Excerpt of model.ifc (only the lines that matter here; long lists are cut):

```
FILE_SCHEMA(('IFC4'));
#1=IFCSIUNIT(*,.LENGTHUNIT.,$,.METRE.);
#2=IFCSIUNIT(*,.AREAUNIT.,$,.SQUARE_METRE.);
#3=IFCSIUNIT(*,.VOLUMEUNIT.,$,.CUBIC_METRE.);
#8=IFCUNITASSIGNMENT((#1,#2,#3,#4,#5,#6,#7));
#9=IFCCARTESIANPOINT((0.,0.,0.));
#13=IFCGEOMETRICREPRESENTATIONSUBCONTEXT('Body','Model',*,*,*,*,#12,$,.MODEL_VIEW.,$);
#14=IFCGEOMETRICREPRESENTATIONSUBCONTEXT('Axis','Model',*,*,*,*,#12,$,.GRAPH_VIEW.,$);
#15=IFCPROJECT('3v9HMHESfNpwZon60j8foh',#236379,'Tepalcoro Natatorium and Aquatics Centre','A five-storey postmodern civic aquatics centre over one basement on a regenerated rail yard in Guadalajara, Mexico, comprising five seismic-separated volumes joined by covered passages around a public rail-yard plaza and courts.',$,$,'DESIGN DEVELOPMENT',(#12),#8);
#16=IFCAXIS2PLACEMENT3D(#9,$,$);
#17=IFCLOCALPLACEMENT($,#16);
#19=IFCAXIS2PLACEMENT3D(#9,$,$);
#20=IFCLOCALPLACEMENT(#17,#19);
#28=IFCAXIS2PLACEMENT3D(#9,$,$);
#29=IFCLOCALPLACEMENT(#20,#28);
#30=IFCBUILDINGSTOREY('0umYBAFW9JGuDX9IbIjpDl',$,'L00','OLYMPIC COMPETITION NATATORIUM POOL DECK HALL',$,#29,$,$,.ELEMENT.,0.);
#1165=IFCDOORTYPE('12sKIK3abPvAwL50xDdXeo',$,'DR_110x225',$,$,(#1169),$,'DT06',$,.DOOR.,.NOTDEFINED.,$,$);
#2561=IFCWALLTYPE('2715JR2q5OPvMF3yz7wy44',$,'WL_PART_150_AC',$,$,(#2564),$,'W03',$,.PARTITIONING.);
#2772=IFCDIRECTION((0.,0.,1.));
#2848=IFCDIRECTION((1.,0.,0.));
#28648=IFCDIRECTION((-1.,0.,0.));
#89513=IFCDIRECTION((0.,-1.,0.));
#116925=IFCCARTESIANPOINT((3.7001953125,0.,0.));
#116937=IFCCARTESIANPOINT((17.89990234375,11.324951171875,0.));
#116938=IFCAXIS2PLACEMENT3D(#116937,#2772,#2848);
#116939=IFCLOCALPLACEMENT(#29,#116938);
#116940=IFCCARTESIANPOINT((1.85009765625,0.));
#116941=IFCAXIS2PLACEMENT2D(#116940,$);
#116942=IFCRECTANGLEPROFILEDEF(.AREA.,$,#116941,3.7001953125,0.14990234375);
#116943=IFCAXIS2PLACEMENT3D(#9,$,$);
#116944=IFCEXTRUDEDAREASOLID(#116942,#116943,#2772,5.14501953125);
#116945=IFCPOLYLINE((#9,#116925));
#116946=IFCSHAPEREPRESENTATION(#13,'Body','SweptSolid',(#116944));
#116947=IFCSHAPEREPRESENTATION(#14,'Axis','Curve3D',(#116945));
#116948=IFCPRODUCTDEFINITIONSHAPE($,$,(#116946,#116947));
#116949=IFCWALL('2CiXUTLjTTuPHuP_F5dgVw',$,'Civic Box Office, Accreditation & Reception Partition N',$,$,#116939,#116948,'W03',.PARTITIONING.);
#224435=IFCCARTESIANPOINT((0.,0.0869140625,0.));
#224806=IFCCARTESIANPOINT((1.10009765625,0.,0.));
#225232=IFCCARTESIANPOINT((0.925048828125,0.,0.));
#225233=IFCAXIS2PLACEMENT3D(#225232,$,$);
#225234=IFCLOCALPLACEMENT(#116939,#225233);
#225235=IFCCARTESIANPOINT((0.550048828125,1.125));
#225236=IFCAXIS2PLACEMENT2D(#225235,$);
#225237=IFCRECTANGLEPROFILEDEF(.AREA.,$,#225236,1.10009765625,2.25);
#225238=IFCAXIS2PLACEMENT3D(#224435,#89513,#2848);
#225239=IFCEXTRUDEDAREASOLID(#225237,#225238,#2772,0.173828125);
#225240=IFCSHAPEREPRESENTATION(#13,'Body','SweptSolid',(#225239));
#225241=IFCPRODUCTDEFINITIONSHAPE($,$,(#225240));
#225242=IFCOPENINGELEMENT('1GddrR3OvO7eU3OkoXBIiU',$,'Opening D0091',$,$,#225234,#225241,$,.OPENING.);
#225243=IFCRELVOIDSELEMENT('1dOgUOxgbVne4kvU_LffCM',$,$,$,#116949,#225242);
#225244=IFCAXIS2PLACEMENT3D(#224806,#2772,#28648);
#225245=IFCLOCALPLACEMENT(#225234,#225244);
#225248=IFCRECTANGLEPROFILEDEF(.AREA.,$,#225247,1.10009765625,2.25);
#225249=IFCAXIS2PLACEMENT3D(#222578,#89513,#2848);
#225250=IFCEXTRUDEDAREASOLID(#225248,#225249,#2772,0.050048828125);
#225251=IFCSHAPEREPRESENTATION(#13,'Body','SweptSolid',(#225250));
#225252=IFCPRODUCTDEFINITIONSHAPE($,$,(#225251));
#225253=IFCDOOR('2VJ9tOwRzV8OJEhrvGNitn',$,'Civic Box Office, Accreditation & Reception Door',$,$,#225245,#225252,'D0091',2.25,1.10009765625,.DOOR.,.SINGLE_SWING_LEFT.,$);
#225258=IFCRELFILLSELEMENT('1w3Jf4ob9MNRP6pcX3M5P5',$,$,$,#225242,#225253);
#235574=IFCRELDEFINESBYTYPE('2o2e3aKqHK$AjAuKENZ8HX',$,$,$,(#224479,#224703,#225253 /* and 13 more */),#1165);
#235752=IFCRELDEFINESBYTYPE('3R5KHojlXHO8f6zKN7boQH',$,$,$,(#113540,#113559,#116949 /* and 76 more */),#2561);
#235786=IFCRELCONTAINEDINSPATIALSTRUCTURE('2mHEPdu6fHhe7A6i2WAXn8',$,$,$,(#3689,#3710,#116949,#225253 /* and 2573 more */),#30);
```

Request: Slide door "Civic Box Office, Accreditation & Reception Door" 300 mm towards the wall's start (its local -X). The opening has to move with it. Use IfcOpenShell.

```python
import ifcopenshell
import ifcopenshell.api.geometry
import ifcopenshell.util.placement
import ifcopenshell.util.unit

model = ifcopenshell.open("model.ifc")
unit_scale = ifcopenshell.util.unit.calculate_unit_scale(model)

door = model.by_id(225253)
opening = door.FillsVoids[0].RelatingOpeningElement
wall = opening.VoidsElements[0].RelatingBuildingElement

wall_matrix = ifcopenshell.util.placement.get_local_placement(wall.ObjectPlacement)
shift = wall_matrix[:3, 0] * -0.3 / unit_scale
before = ifcopenshell.util.placement.get_local_placement(door.ObjectPlacement)[:3, 3].copy()

# The door is placed relative to its opening, so it follows when the opening moves.
matrix = ifcopenshell.util.placement.get_local_placement(opening.ObjectPlacement)
matrix[:3, 3] += shift
ifcopenshell.api.geometry.edit_object_placement(
    model, product=opening, matrix=matrix, is_si=False, should_transform_children=True
)

after = ifcopenshell.util.placement.get_local_placement(door.ObjectPlacement)[:3, 3]
print("door moved by", (after - before).round(3) + 0.0)

model.write("model_edited.ifc")
```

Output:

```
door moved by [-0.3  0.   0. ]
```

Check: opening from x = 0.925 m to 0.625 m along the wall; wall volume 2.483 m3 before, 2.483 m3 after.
